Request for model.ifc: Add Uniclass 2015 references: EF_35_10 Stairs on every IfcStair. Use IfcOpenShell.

First a look at what the model holds.

```python
import ifcopenshell

model = ifcopenshell.open("model.ifc")
print(model.schema)
print("classifications:", [c.Name for c in model.by_type("IfcClassification")])
for ifc_class in ("IfcDoor", "IfcRoof", "IfcStair", "IfcWall", "IfcWindow"):
    print(ifc_class, len(model.by_type(ifc_class)))
```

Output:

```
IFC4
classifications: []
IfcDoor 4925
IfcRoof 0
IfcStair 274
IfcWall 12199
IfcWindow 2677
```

```python
import ifcopenshell
import ifcopenshell.api.classification

model = ifcopenshell.open("model.ifc")

system = ifcopenshell.api.classification.add_classification(model, classification="Uniclass 2015")

codes = {
    "IfcStair": ("EF_35_10", "Stairs"),
}
for ifc_class, (code, name) in codes.items():
    products = model.by_type(ifc_class)
    ifcopenshell.api.classification.add_reference(
        model, products=products, classification=system, identification=code, name=name
    )
    print(code, len(products))

model.write("model_rev.ifc")
```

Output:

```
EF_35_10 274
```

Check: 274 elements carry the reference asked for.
